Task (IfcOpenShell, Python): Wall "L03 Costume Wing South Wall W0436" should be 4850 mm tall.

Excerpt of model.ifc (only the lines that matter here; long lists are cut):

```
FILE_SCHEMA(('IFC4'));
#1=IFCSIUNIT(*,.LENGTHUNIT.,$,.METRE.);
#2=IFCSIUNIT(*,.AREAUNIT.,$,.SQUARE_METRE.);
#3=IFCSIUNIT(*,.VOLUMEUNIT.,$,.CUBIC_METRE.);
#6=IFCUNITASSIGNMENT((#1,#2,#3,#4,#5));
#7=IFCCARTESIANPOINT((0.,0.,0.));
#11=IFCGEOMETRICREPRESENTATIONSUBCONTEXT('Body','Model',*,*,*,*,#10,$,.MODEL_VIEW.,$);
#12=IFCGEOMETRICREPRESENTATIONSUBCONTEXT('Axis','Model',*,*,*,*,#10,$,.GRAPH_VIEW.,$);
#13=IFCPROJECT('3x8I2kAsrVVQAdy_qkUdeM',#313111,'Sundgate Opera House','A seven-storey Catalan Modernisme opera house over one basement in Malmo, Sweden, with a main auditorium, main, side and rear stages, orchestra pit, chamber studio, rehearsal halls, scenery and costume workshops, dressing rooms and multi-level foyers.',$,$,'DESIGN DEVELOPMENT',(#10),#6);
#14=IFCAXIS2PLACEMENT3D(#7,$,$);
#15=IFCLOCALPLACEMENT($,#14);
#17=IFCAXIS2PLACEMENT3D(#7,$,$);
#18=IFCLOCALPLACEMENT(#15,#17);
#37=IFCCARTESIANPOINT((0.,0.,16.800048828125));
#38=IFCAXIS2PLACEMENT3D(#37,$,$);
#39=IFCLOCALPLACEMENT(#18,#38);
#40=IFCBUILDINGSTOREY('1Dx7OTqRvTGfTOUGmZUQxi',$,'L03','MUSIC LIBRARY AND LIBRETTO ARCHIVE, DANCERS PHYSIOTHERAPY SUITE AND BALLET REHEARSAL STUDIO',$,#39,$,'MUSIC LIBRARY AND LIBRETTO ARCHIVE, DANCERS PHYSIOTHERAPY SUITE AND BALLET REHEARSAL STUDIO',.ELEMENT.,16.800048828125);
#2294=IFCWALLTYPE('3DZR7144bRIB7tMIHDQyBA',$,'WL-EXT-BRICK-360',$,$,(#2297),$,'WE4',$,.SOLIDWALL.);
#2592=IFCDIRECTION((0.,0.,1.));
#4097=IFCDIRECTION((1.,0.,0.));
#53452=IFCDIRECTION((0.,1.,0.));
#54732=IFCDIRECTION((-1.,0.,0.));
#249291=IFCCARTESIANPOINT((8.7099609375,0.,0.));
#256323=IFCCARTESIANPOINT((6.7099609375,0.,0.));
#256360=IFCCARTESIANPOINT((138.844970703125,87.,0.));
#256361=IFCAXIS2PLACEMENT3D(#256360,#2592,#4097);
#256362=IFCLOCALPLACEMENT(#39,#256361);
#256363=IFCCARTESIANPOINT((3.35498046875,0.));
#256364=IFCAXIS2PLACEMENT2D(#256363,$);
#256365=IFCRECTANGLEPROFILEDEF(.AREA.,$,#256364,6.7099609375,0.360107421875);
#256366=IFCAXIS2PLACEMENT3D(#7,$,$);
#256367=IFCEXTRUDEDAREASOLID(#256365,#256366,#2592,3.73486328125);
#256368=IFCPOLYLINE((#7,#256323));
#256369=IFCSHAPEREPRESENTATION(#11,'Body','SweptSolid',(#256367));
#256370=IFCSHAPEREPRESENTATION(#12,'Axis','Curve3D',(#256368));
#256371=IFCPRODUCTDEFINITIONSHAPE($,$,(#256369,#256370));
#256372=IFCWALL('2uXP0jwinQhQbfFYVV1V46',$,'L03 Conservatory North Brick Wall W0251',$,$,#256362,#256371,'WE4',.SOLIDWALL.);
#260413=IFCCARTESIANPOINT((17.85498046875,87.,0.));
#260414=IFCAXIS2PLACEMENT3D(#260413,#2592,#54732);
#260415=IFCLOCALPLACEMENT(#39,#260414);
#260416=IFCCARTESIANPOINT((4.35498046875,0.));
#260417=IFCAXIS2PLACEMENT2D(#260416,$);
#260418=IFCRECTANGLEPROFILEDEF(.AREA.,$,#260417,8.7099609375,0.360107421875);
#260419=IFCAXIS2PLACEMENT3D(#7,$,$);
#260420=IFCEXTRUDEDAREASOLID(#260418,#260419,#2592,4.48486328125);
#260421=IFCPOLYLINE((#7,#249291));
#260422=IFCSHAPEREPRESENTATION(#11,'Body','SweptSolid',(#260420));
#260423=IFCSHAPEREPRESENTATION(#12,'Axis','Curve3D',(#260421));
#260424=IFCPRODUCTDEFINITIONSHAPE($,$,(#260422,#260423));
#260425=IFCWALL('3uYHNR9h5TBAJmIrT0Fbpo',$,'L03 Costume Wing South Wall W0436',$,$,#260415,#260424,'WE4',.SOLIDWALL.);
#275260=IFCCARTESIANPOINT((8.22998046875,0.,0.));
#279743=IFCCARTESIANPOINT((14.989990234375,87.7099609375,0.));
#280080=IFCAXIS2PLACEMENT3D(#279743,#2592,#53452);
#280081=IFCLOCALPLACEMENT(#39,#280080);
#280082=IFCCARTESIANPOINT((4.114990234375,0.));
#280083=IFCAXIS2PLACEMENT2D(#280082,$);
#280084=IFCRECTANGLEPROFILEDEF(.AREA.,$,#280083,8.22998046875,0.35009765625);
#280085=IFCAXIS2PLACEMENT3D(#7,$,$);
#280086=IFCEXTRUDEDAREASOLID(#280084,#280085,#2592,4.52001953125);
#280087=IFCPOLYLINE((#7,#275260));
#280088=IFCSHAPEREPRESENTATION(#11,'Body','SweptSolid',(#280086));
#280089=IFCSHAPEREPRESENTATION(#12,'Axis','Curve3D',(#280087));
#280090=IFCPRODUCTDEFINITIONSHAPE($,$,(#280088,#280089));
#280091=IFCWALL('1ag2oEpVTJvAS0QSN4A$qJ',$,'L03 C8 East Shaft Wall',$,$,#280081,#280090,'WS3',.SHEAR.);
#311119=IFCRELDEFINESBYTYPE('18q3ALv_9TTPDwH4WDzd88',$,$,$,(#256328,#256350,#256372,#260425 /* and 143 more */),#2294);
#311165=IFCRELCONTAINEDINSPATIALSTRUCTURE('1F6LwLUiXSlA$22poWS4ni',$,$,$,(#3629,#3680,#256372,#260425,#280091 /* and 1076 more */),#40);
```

```python
import ifcopenshell
import ifcopenshell.geom
import ifcopenshell.util.representation
import ifcopenshell.util.shape

model = ifcopenshell.open("model.ifc")
settings = ifcopenshell.geom.settings()


def volume(element):
    """Net volume in cubic metres, openings subtracted."""
    shape = ifcopenshell.geom.create_shape(settings, element)
    return ifcopenshell.util.shape.get_volume(shape.geometry)


wall = model.by_guid("3uYHNR9h5TBAJmIrT0Fbpo")
before = volume(wall)

body = ifcopenshell.util.representation.get_representation(wall, "Model", "Body")
solid = body.Items[0]
old_height = solid.Depth
solid.Depth = 4.85
after = volume(wall)

print(f"height {old_height:g} -> {solid.Depth:g}, volume {before:.3f} -> {after:.3f} m3")

model.write("model_v2.ifc")
```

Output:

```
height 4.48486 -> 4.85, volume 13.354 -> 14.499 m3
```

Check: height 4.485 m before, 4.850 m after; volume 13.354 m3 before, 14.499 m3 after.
